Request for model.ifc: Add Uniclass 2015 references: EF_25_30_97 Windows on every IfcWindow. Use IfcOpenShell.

First a look at what the model holds.

```python
import ifcopenshell

model = ifcopenshell.open("model.ifc")
print(model.schema)
print("classifications:", [c.Name for c in model.by_type("IfcClassification")])
for ifc_class in ("IfcDoor", "IfcRoof", "IfcStair", "IfcWall", "IfcWindow"):
    print(ifc_class, len(model.by_type(ifc_class)))
```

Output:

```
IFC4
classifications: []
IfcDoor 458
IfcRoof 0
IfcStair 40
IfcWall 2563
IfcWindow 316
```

```python
import ifcopenshell
import ifcopenshell.api.classification

model = ifcopenshell.open("model.ifc")

system = ifcopenshell.api.classification.add_classification(model, classification="Uniclass 2015")

codes = {
    "IfcWindow": ("EF_25_30_97", "Windows"),
}
for ifc_class, (code, name) in codes.items():
    products = model.by_type(ifc_class)
    ifcopenshell.api.classification.add_reference(
        model, products=products, classification=system, identification=code, name=name
    )
    print(code, len(products))

model.write("model_v2.ifc")
```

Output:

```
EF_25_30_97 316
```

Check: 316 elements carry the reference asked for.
